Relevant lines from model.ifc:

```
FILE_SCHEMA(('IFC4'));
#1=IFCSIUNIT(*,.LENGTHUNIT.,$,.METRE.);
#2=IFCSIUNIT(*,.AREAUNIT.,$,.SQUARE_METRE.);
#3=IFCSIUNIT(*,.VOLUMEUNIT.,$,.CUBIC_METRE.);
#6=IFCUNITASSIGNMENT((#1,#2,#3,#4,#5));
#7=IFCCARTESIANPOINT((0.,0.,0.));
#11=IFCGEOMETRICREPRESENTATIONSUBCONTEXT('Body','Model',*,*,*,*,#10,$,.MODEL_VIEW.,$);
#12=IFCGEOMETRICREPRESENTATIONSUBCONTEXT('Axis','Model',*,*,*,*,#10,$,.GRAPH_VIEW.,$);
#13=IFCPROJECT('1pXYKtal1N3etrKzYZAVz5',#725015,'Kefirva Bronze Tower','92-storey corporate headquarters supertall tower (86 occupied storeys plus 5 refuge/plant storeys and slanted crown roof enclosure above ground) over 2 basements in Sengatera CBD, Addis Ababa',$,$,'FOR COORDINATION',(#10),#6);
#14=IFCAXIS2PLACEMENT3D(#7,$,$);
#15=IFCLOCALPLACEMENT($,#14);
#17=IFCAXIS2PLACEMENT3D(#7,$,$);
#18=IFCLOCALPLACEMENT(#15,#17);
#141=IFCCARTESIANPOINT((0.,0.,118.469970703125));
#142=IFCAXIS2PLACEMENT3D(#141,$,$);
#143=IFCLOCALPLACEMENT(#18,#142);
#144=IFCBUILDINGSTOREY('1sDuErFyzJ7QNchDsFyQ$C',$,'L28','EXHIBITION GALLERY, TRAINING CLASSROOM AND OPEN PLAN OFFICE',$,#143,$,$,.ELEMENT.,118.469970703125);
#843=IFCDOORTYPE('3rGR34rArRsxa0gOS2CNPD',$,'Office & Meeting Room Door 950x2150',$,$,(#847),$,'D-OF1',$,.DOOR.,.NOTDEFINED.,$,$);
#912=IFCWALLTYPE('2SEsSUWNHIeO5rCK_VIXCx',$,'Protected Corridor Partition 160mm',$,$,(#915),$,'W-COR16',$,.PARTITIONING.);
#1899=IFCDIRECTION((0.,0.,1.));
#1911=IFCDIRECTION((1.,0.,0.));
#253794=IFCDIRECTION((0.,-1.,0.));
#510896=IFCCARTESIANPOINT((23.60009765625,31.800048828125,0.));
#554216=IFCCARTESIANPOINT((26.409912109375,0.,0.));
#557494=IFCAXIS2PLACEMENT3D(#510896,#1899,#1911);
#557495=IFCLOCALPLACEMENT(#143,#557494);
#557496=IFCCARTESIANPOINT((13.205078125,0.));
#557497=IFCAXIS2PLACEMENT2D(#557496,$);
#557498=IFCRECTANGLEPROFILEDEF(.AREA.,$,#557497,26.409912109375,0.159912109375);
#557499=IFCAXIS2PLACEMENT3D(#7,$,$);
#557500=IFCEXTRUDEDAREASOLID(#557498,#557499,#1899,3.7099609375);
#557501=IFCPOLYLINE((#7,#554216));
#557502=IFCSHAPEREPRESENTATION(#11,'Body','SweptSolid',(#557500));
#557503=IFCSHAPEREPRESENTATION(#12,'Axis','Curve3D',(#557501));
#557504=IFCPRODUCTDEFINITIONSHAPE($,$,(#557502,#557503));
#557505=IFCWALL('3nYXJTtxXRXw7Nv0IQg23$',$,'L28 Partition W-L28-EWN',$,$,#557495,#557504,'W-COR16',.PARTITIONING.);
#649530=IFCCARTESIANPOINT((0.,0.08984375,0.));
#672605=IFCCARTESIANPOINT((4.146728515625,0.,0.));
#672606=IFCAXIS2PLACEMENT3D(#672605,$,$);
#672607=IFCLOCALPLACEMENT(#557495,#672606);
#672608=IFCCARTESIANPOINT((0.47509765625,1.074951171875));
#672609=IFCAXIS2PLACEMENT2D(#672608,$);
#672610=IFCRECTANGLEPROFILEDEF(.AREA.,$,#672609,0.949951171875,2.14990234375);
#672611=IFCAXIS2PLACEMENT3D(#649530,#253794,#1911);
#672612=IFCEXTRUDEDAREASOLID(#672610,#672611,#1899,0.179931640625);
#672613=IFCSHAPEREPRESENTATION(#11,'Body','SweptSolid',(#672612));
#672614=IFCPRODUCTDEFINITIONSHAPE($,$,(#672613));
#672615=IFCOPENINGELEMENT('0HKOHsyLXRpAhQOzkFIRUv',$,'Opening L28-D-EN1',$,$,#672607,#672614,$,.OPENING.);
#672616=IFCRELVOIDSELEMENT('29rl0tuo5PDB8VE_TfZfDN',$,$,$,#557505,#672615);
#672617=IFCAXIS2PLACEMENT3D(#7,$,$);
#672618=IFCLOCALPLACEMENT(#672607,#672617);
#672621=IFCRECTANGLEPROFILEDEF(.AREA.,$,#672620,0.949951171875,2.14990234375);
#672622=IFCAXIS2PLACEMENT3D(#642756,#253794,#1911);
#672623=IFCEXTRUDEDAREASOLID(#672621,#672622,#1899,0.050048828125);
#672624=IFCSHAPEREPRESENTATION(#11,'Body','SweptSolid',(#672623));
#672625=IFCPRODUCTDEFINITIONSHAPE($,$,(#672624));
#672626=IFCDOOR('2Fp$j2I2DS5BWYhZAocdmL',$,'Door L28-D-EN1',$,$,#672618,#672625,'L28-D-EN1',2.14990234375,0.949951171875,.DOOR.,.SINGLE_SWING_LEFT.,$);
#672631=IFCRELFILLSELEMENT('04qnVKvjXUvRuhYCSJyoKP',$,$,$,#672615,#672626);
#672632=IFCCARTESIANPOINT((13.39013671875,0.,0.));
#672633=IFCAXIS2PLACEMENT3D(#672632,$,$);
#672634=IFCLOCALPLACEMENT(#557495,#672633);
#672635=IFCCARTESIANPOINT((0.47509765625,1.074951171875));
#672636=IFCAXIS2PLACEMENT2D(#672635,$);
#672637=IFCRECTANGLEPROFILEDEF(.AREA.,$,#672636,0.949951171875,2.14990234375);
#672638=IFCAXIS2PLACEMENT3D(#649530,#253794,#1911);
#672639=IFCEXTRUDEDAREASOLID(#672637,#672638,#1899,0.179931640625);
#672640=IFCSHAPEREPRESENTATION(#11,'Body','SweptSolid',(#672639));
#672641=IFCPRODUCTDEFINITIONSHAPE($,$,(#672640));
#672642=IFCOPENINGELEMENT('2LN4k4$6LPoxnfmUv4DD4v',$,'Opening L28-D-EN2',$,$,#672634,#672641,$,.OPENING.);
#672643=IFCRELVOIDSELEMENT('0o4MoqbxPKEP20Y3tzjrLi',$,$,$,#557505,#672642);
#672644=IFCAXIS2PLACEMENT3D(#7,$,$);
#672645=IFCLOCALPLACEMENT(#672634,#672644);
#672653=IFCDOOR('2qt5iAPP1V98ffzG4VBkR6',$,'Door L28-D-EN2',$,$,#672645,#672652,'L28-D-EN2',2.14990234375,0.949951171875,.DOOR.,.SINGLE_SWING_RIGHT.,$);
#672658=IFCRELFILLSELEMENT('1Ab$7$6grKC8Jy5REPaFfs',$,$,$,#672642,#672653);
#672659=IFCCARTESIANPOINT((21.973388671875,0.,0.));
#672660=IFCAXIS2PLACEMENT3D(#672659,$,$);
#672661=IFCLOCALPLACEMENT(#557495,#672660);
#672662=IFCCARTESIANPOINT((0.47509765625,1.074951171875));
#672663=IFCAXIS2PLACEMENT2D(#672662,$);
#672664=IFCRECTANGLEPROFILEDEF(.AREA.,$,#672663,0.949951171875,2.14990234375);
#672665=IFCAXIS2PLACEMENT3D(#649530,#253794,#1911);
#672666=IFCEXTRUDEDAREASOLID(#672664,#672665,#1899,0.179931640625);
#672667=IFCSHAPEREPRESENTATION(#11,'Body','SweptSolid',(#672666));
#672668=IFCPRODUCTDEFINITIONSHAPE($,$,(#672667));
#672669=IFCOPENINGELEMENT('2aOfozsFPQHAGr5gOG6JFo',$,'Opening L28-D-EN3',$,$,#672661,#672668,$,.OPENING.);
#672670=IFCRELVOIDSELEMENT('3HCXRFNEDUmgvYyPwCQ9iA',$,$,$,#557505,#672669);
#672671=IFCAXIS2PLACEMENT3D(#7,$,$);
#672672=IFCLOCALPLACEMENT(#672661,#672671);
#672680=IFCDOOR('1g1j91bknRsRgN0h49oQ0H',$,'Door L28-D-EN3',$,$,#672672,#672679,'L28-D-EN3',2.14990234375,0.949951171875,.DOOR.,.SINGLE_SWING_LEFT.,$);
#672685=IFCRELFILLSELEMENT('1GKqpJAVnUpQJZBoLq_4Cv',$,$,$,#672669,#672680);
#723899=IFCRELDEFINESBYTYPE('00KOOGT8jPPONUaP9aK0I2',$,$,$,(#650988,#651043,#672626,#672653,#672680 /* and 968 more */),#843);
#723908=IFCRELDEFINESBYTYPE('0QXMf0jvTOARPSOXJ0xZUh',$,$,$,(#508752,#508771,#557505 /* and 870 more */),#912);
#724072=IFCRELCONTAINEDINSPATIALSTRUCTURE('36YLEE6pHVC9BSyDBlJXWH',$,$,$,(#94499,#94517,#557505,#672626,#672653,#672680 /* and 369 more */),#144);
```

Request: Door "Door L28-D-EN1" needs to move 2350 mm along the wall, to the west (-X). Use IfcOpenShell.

```python
import ifcopenshell
import ifcopenshell.api.geometry
import ifcopenshell.util.placement

model = ifcopenshell.open("model.ifc")

door = model.by_id(672626)
opening = door.FillsVoids[0].RelatingOpeningElement
wall = opening.VoidsElements[0].RelatingBuildingElement

wall_matrix = ifcopenshell.util.placement.get_local_placement(wall.ObjectPlacement)
shift = wall_matrix[:3, 0] * -2.35
before = ifcopenshell.util.placement.get_local_placement(door.ObjectPlacement)[:3, 3].copy()

# The door is placed relative to its opening, so it follows when the opening moves.
matrix = ifcopenshell.util.placement.get_local_placement(opening.ObjectPlacement)
matrix[:3, 3] += shift
ifcopenshell.api.geometry.edit_object_placement(
    model, product=opening, matrix=matrix, is_si=False, should_transform_children=True
)

after = ifcopenshell.util.placement.get_local_placement(door.ObjectPlacement)[:3, 3]
print("door moved by", (after - before).round(3) + 0.0)

model.write("model_updated.ifc")
```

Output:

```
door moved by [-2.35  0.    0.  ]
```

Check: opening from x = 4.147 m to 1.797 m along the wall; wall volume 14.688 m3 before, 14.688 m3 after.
